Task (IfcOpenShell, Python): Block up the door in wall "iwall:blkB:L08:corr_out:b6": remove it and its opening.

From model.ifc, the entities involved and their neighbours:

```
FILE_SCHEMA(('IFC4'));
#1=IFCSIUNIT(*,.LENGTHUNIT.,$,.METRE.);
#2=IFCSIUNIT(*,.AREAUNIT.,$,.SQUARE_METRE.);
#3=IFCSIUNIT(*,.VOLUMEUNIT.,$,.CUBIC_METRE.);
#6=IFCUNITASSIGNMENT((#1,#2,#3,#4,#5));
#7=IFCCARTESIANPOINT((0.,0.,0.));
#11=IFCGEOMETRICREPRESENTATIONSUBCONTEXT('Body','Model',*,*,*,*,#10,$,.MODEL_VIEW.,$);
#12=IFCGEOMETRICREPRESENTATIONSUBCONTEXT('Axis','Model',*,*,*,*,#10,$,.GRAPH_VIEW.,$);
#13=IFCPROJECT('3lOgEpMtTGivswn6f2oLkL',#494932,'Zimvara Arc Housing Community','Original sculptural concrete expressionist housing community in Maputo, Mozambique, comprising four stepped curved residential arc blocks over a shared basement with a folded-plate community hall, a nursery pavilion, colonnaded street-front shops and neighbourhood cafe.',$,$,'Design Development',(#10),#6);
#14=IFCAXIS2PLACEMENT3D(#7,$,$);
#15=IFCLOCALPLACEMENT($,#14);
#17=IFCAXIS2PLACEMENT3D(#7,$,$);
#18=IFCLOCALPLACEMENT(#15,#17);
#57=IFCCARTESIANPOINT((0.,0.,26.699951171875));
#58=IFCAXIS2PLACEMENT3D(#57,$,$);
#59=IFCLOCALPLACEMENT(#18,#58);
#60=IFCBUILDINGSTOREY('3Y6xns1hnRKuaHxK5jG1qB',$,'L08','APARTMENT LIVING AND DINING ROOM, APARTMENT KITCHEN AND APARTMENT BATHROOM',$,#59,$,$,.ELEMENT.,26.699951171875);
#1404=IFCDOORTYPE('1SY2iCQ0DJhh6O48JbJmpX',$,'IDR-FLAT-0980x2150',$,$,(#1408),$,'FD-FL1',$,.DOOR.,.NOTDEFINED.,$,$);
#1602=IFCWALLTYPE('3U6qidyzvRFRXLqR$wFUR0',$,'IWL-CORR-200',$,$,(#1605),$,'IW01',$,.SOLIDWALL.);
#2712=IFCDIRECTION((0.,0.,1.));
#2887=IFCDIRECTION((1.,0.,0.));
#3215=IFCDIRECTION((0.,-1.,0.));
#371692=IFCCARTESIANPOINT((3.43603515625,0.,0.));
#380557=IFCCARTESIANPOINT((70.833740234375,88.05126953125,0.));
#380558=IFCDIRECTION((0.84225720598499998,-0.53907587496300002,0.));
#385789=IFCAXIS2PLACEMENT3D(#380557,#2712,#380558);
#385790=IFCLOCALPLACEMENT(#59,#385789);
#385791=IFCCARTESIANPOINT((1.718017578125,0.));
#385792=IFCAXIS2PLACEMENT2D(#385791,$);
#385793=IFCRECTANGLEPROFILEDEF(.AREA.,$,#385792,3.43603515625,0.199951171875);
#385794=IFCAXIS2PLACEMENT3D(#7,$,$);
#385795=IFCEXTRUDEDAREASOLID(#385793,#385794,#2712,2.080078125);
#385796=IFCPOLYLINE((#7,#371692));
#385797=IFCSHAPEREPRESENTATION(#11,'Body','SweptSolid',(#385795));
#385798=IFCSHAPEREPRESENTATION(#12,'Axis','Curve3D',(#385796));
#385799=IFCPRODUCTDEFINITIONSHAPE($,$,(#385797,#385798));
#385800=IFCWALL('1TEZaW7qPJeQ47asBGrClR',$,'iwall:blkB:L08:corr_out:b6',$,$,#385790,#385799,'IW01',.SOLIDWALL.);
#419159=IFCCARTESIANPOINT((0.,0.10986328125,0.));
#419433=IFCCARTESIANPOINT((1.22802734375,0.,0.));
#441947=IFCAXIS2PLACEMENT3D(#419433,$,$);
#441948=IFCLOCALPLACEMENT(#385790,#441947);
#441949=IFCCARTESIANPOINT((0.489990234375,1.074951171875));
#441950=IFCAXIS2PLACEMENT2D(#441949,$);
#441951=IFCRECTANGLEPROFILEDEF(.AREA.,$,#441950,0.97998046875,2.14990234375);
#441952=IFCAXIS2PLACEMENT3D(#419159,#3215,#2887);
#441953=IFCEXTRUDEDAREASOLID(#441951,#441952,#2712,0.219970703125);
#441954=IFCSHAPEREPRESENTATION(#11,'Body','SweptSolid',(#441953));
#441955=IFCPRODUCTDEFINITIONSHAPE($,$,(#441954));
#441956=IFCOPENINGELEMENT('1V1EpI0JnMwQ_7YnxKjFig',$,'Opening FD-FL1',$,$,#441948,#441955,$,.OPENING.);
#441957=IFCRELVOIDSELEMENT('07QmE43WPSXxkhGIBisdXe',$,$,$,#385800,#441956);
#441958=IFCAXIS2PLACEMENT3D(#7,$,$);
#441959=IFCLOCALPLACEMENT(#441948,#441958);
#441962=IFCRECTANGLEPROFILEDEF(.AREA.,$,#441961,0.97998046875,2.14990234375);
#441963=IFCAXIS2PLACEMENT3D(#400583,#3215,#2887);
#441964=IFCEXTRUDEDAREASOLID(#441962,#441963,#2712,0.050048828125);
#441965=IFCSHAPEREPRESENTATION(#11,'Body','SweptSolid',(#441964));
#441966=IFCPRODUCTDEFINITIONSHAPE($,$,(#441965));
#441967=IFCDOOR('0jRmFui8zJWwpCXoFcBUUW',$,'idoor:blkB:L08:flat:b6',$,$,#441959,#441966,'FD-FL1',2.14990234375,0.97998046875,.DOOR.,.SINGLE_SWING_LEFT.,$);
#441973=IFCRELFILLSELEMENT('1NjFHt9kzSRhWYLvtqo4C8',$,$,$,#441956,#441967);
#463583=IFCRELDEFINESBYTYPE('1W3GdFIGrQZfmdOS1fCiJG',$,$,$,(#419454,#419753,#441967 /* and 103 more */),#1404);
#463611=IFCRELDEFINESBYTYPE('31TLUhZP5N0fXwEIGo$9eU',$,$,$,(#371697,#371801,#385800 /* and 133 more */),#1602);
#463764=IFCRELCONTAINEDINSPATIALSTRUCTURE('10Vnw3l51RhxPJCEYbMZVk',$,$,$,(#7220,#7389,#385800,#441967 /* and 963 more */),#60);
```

```python
import ifcopenshell
import ifcopenshell.api.feature
import ifcopenshell.api.root
import ifcopenshell.geom
import ifcopenshell.util.shape

model = ifcopenshell.open("model.ifc")
settings = ifcopenshell.geom.settings()


def volume(element):
    """Net volume in cubic metres, openings subtracted."""
    shape = ifcopenshell.geom.create_shape(settings, element)
    return ifcopenshell.util.shape.get_volume(shape.geometry)


door = model.by_guid("0jRmFui8zJWwpCXoFcBUUW")
opening = door.FillsVoids[0].RelatingOpeningElement
wall = opening.VoidsElements[0].RelatingBuildingElement
before = volume(wall)

ifcopenshell.api.root.remove_product(model, product=door)
ifcopenshell.api.feature.remove_feature(model, feature=opening)

after = volume(wall)

print(f"wall volume {before:.3f} -> {after:.3f} m3")

model.write("model_v2.ifc")
```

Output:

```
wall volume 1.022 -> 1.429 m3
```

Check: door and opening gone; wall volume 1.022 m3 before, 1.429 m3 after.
